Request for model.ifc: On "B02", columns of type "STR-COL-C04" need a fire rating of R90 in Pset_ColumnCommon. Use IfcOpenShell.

First a look at what the model holds.

```python
import ifcopenshell
import ifcopenshell.util.element

model = ifcopenshell.open("model.ifc")
print(model.schema)
storey = next(s for s in model.by_type("IfcBuildingStorey") if s.Name == "B02")
columns = [e for e in ifcopenshell.util.element.get_decomposition(storey) if e.is_a("IfcColumn")]
seen = {}
for e in columns:
    element_type = ifcopenshell.util.element.get_type(e)
    key = (element_type.Name if element_type != e and element_type else None, ifcopenshell.util.element.get_pset(e, "Pset_ColumnCommon", "FireRating"))
    seen[key] = seen.get(key, 0) + 1
for (name, value), count in sorted(seen.items(), key=str):
    print(count, "x", name, "|", value)
```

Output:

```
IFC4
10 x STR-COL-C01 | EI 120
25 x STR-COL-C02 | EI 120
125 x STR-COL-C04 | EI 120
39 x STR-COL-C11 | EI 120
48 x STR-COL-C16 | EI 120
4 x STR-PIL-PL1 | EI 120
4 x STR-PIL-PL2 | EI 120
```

```python
import ifcopenshell
import ifcopenshell.api.pset
import ifcopenshell.util.element

model = ifcopenshell.open("model.ifc")

storey = next(s for s in model.by_type("IfcBuildingStorey") if s.Name == "B02")
columns = [e for e in ifcopenshell.util.element.get_decomposition(storey) if e.is_a("IfcColumn")]

count = 0
for e in columns:
    element_type = ifcopenshell.util.element.get_type(e)
    if element_type in (None, e) or element_type.Name != "STR-COL-C04":
        continue
    # add_pset returns the element's existing set when there is one.
    pset = ifcopenshell.api.pset.add_pset(model, product=e, name="Pset_ColumnCommon")
    ifcopenshell.api.pset.edit_pset(model, pset=pset, properties={"FireRating": "R90"})
    count += 1

print(count, "columns updated")

model.write("model_updated.ifc")
```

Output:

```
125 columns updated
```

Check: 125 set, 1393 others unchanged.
